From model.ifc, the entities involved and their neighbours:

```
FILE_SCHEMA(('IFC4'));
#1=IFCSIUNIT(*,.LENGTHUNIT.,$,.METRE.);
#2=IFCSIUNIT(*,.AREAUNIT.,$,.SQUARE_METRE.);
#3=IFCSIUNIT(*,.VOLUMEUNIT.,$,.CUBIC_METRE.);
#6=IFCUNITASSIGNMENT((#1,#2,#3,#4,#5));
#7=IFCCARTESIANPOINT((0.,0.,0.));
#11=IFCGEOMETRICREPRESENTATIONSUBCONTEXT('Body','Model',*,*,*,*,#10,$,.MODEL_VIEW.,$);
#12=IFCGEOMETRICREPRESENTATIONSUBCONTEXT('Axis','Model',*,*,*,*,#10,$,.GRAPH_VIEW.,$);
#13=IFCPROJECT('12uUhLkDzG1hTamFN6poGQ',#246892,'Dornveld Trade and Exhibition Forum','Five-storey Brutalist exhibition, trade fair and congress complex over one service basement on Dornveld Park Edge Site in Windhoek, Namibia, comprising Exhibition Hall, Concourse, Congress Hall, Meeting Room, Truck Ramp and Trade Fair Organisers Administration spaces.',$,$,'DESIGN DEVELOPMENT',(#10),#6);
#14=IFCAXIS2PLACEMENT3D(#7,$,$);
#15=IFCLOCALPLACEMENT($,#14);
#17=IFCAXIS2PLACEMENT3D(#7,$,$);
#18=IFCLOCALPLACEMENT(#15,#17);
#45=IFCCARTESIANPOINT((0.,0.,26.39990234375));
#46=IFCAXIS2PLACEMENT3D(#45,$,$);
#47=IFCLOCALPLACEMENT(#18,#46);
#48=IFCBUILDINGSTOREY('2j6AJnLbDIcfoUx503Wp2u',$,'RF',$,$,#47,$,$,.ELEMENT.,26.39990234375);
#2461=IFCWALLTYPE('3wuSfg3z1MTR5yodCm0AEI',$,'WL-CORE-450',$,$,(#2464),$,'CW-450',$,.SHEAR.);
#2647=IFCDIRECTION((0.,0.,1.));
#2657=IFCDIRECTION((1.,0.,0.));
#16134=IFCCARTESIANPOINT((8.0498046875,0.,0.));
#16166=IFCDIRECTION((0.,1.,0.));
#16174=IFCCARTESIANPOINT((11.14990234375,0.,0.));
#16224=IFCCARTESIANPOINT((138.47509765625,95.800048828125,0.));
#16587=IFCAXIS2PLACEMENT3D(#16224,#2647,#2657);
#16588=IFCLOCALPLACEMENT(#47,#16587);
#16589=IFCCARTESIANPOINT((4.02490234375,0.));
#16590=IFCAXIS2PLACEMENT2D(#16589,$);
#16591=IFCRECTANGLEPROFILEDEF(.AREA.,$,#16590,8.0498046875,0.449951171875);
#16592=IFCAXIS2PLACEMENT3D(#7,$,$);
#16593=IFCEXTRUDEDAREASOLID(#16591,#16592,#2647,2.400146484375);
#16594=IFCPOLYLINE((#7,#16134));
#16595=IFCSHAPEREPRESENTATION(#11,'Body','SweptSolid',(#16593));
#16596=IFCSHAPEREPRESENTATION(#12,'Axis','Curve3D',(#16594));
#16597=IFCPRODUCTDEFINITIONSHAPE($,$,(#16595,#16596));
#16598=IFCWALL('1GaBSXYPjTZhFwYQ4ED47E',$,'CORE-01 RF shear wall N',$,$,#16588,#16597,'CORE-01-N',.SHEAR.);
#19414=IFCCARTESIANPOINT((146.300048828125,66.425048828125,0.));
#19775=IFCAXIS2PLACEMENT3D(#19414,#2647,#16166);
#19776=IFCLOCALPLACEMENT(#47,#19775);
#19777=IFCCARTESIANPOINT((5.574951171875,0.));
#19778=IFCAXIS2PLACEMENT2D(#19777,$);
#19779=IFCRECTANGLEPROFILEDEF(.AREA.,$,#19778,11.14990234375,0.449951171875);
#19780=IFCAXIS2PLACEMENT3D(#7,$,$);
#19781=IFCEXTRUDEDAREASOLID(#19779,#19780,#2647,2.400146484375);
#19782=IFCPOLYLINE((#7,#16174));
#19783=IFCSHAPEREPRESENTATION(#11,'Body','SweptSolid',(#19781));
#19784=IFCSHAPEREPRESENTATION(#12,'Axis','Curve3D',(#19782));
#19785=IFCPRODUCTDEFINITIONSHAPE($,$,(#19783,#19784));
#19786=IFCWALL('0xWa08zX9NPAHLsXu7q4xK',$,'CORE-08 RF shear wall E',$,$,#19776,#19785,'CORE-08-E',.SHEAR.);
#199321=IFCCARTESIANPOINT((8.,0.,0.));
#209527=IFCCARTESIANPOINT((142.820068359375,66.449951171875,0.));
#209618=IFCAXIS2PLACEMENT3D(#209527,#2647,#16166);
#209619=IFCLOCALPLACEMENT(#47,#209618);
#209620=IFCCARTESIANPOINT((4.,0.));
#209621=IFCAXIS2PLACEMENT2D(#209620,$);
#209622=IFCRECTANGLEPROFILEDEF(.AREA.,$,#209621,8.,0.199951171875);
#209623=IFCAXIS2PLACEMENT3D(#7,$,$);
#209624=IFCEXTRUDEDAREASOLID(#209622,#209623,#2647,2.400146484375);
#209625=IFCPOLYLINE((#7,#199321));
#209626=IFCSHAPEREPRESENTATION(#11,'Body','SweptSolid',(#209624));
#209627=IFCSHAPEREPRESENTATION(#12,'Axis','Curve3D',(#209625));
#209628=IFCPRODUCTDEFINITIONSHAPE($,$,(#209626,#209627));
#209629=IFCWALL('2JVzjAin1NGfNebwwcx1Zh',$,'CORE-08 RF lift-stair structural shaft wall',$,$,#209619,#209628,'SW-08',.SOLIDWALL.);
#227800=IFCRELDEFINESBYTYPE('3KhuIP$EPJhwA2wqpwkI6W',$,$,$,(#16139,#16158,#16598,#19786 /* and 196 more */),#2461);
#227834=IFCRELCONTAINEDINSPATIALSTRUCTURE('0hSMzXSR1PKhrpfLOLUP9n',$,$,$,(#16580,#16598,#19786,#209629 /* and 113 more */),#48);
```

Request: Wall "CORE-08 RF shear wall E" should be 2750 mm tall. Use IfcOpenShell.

```python
import ifcopenshell
import ifcopenshell.geom
import ifcopenshell.util.representation
import ifcopenshell.util.shape

model = ifcopenshell.open("model.ifc")
settings = ifcopenshell.geom.settings()


def volume(element):
    """Net volume in cubic metres, openings subtracted."""
    shape = ifcopenshell.geom.create_shape(settings, element)
    return ifcopenshell.util.shape.get_volume(shape.geometry)


wall = model.by_id(19786)
before = volume(wall)

body = ifcopenshell.util.representation.get_representation(wall, "Model", "Body")
solid = body.Items[0]
old_height = solid.Depth
solid.Depth = 2.75
after = volume(wall)

print(f"height {old_height:g} -> {solid.Depth:g}, volume {before:.3f} -> {after:.3f} m3")

model.write("model_rev.ifc")
```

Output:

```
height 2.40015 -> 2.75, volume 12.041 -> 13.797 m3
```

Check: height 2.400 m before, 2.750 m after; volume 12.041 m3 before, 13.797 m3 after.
